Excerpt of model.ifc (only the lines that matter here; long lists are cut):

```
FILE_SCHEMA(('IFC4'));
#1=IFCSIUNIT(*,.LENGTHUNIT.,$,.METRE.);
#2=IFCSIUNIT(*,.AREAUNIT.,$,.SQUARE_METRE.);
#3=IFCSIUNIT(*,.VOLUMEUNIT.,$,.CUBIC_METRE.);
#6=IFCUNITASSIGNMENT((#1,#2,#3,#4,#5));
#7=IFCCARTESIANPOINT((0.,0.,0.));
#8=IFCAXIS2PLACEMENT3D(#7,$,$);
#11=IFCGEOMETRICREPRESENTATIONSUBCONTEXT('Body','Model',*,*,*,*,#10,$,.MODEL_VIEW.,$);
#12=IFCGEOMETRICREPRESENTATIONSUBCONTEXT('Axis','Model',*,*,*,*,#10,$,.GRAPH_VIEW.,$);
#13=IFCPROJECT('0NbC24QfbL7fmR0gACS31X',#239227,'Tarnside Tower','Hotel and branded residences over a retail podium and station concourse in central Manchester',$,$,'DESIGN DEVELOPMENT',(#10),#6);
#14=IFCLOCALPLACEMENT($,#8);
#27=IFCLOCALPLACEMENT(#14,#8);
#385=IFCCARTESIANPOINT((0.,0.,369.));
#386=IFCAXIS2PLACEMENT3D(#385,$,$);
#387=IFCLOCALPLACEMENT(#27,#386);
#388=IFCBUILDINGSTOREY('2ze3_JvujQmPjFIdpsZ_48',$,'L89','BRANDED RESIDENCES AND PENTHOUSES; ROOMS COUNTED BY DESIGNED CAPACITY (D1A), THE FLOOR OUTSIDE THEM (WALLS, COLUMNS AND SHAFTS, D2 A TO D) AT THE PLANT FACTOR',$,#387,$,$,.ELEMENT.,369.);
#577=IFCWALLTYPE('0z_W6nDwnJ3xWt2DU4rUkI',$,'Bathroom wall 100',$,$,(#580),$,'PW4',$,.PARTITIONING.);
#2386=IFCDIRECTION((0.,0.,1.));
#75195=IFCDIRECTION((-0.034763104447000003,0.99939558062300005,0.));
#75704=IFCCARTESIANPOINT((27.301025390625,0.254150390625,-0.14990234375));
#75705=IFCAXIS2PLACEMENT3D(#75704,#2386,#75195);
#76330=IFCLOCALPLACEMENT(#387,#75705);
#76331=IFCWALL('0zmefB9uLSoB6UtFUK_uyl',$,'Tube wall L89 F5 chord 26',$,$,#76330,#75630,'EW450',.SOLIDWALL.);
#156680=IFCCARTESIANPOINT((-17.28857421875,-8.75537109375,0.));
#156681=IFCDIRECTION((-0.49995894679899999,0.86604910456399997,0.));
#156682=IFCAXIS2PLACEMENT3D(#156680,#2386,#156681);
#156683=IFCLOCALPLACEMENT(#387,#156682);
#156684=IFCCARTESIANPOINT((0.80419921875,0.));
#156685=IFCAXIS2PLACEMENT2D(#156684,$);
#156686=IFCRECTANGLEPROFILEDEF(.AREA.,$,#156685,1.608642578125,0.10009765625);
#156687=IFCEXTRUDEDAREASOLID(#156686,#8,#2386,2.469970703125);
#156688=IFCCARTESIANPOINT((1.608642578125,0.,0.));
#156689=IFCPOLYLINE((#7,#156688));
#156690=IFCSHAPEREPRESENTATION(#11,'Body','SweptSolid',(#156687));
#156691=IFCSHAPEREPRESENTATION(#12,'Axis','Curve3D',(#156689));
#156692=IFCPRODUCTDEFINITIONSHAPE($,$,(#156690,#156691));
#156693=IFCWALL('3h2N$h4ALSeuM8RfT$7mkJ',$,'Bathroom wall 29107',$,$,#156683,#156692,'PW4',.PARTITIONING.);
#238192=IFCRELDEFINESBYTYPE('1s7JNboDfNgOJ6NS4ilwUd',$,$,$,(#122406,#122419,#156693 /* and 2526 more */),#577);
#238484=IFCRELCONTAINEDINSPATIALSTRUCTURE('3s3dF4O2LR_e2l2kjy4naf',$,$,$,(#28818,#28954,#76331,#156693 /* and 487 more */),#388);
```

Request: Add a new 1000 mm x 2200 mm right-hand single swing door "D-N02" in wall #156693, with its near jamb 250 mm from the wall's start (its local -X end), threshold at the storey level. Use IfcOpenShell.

```python
import numpy as np
import ifcopenshell
import ifcopenshell.api.feature
import ifcopenshell.api.geometry
import ifcopenshell.api.root
import ifcopenshell.api.spatial
import ifcopenshell.geom
import ifcopenshell.util.element
import ifcopenshell.util.placement
import ifcopenshell.util.representation
import ifcopenshell.util.shape
import ifcopenshell.util.unit

model = ifcopenshell.open("model.ifc")
unit_scale = ifcopenshell.util.unit.calculate_unit_scale(model)
settings = ifcopenshell.geom.settings()


def volume(element):
    """Net volume in cubic metres, openings subtracted."""
    shape = ifcopenshell.geom.create_shape(settings, element)
    return ifcopenshell.util.shape.get_volume(shape.geometry)


wall = model.by_guid("3h2N$h4ALSeuM8RfT$7mkJ")
storey = ifcopenshell.util.element.get_container(wall, ifc_class="IfcBuildingStorey")
context = ifcopenshell.util.representation.get_context(model, "Model", "Body", "MODEL_VIEW")
before = volume(wall)

width, height, from_end, sill = 1, 2.2, 0.25, 0.0  # metres

# The wall runs along its own X axis, and the end named is its -X end.
wall_shape = ifcopenshell.geom.create_shape(settings, wall)
x, y, z = ifcopenshell.util.shape.get_vertices(wall_shape.geometry).T
start = x.min() + from_end
face, thickness = float(y.min()), float(y.max() - y.min())
wall_matrix = ifcopenshell.util.placement.get_local_placement(wall.ObjectPlacement)
level = ifcopenshell.util.placement.get_local_placement(storey.ObjectPlacement)[2, 3]


def in_wall(x, y):
    """Placement at x, y metres in the wall's axes, at sill height."""
    matrix = wall_matrix.copy()
    matrix[:, 3] = wall_matrix @ np.array([x / unit_scale, y / unit_scale, 0.0, 1.0])
    matrix[2, 3] = level + sill / unit_scale
    return matrix


# Opening: a box that overshoots both wall faces by 50 mm.
opening = ifcopenshell.api.root.create_entity(model, ifc_class="IfcOpeningElement", predefined_type="OPENING")
box = ifcopenshell.api.geometry.add_wall_representation(
    model, context=context, length=width, height=height, thickness=thickness + 0.1
)
ifcopenshell.api.geometry.assign_representation(model, product=opening, representation=box)
ifcopenshell.api.geometry.edit_object_placement(model, product=opening, matrix=in_wall(start, face - 0.05), is_si=False)
ifcopenshell.api.feature.add_feature(model, feature=opening, element=wall)

door = ifcopenshell.api.root.create_entity(model, ifc_class="IfcDoor", name="D-N02", predefined_type="DOOR")
door.OverallWidth, door.OverallHeight = width / unit_scale, height / unit_scale
door.OperationType = "SINGLE_SWING_RIGHT"
body = ifcopenshell.api.geometry.add_door_representation(
    model,
    context=context,
    overall_width=door.OverallWidth,
    overall_height=door.OverallHeight,
    operation_type="SINGLE_SWING_RIGHT",
    lining_properties={"LiningDepth": thickness / unit_scale, "ThresholdDepth": thickness / unit_scale},
)
ifcopenshell.api.geometry.assign_representation(model, product=door, representation=body)
ifcopenshell.api.spatial.assign_container(model, products=[door], relating_structure=storey)
ifcopenshell.api.feature.add_filling(model, opening=opening, element=door)

# The lining spans the wall, so the door starts at the wall face.
ifcopenshell.api.geometry.edit_object_placement(model, product=door, matrix=in_wall(start, face), is_si=False)

after = volume(wall)

print(f"wall volume {before:.3f} -> {after:.3f} m3")

model.write("model_updated.ifc")
```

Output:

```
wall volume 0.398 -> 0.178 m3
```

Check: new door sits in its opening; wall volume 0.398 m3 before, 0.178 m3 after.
